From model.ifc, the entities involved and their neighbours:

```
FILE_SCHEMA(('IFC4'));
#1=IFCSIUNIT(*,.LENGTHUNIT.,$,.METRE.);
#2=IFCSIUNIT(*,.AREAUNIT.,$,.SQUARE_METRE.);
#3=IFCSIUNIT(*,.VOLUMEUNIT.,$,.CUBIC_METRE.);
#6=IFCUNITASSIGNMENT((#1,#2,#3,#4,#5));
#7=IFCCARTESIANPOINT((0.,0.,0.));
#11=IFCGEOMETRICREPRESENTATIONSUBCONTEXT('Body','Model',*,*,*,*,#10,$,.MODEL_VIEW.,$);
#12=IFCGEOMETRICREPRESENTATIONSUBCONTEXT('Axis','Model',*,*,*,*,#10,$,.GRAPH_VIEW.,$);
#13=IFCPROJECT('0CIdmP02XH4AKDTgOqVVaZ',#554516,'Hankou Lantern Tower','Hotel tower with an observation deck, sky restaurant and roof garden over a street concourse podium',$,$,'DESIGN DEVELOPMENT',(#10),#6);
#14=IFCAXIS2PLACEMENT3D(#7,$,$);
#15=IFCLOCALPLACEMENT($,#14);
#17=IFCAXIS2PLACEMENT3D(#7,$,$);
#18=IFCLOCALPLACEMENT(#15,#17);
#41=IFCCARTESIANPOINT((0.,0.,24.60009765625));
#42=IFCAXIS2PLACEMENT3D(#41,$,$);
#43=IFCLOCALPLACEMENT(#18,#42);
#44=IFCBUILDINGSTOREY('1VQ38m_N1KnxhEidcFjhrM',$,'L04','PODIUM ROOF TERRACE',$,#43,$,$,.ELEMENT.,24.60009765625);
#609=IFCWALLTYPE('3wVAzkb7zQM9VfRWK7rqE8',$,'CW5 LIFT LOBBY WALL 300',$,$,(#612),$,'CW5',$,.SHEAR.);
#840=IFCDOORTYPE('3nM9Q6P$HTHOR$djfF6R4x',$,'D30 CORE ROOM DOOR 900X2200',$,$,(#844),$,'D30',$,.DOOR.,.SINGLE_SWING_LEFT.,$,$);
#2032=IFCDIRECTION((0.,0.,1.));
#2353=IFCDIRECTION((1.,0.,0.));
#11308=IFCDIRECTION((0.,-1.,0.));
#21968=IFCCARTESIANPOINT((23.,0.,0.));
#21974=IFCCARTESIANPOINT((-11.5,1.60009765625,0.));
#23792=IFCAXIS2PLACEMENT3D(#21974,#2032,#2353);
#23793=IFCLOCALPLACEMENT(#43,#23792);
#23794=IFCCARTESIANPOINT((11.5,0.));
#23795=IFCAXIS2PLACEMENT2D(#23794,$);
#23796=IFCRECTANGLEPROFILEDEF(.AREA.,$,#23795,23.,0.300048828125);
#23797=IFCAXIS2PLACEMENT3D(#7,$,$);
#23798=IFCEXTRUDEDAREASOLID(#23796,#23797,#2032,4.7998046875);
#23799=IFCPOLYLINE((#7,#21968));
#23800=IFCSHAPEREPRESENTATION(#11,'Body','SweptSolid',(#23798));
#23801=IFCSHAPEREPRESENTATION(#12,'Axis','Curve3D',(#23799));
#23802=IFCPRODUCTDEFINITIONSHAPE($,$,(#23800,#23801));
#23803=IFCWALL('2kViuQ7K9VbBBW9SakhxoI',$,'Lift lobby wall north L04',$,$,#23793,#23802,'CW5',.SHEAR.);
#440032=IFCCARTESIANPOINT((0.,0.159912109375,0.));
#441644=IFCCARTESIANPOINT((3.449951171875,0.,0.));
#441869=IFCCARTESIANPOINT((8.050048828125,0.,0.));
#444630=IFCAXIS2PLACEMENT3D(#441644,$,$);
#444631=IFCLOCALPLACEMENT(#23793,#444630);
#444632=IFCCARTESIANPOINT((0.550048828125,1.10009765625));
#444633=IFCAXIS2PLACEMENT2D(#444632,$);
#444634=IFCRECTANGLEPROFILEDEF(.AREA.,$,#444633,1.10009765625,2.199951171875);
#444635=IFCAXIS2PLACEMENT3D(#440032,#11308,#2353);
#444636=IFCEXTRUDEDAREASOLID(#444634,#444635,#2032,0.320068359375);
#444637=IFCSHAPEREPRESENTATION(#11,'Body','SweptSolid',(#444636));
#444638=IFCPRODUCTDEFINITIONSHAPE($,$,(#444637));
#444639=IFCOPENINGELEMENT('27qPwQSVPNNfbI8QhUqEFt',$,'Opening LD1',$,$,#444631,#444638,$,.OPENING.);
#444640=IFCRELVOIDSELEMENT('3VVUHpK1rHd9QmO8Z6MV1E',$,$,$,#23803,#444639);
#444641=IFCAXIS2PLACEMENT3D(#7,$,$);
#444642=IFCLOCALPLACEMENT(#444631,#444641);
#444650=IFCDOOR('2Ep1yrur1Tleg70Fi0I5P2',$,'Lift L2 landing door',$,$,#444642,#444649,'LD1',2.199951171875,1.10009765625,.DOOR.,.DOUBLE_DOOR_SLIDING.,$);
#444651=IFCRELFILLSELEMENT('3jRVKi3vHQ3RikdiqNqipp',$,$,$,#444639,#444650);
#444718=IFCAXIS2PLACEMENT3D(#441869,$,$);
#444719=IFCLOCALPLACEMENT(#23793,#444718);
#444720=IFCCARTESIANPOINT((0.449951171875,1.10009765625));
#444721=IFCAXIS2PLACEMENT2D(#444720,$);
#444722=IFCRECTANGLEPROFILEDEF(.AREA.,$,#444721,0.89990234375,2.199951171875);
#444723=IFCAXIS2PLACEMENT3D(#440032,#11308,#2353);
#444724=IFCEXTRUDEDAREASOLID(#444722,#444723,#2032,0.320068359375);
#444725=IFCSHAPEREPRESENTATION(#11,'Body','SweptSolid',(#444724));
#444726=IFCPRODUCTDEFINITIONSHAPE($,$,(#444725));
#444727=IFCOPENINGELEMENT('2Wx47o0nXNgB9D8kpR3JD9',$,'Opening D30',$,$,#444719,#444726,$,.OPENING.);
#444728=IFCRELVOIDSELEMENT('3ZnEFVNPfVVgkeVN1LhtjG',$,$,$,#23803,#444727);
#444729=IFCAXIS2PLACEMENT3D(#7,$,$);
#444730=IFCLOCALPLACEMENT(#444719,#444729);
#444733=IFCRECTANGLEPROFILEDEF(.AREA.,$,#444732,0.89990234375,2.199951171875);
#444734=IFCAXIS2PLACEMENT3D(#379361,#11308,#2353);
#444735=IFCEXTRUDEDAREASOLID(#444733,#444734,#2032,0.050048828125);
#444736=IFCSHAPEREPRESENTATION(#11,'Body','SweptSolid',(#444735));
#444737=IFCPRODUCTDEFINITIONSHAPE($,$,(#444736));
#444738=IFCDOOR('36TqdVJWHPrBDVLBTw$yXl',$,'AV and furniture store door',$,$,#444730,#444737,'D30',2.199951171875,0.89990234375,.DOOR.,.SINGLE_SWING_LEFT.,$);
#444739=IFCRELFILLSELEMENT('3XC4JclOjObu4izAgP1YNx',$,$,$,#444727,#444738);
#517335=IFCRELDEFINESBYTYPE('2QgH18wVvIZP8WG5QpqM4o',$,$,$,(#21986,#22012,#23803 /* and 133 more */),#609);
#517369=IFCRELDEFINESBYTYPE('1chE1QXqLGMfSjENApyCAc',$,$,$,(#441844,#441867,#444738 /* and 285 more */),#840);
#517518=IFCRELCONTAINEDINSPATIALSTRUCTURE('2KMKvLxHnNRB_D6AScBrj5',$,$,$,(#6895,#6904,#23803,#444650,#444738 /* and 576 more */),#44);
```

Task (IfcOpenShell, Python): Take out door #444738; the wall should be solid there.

```python
import ifcopenshell
import ifcopenshell.api.feature
import ifcopenshell.api.root
import ifcopenshell.geom
import ifcopenshell.util.shape

model = ifcopenshell.open("model.ifc")
settings = ifcopenshell.geom.settings()


def volume(element):
    """Net volume in cubic metres, openings subtracted."""
    shape = ifcopenshell.geom.create_shape(settings, element)
    return ifcopenshell.util.shape.get_volume(shape.geometry)


door = model.by_guid("36TqdVJWHPrBDVLBTw$yXl")
opening = door.FillsVoids[0].RelatingOpeningElement
wall = opening.VoidsElements[0].RelatingBuildingElement
before = volume(wall)

ifcopenshell.api.root.remove_product(model, product=door)
ifcopenshell.api.feature.remove_feature(model, feature=opening)

after = volume(wall)

print(f"wall volume {before:.3f} -> {after:.3f} m3")

model.write("model_rev.ifc")
```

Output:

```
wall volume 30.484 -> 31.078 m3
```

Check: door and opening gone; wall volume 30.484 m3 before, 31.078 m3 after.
